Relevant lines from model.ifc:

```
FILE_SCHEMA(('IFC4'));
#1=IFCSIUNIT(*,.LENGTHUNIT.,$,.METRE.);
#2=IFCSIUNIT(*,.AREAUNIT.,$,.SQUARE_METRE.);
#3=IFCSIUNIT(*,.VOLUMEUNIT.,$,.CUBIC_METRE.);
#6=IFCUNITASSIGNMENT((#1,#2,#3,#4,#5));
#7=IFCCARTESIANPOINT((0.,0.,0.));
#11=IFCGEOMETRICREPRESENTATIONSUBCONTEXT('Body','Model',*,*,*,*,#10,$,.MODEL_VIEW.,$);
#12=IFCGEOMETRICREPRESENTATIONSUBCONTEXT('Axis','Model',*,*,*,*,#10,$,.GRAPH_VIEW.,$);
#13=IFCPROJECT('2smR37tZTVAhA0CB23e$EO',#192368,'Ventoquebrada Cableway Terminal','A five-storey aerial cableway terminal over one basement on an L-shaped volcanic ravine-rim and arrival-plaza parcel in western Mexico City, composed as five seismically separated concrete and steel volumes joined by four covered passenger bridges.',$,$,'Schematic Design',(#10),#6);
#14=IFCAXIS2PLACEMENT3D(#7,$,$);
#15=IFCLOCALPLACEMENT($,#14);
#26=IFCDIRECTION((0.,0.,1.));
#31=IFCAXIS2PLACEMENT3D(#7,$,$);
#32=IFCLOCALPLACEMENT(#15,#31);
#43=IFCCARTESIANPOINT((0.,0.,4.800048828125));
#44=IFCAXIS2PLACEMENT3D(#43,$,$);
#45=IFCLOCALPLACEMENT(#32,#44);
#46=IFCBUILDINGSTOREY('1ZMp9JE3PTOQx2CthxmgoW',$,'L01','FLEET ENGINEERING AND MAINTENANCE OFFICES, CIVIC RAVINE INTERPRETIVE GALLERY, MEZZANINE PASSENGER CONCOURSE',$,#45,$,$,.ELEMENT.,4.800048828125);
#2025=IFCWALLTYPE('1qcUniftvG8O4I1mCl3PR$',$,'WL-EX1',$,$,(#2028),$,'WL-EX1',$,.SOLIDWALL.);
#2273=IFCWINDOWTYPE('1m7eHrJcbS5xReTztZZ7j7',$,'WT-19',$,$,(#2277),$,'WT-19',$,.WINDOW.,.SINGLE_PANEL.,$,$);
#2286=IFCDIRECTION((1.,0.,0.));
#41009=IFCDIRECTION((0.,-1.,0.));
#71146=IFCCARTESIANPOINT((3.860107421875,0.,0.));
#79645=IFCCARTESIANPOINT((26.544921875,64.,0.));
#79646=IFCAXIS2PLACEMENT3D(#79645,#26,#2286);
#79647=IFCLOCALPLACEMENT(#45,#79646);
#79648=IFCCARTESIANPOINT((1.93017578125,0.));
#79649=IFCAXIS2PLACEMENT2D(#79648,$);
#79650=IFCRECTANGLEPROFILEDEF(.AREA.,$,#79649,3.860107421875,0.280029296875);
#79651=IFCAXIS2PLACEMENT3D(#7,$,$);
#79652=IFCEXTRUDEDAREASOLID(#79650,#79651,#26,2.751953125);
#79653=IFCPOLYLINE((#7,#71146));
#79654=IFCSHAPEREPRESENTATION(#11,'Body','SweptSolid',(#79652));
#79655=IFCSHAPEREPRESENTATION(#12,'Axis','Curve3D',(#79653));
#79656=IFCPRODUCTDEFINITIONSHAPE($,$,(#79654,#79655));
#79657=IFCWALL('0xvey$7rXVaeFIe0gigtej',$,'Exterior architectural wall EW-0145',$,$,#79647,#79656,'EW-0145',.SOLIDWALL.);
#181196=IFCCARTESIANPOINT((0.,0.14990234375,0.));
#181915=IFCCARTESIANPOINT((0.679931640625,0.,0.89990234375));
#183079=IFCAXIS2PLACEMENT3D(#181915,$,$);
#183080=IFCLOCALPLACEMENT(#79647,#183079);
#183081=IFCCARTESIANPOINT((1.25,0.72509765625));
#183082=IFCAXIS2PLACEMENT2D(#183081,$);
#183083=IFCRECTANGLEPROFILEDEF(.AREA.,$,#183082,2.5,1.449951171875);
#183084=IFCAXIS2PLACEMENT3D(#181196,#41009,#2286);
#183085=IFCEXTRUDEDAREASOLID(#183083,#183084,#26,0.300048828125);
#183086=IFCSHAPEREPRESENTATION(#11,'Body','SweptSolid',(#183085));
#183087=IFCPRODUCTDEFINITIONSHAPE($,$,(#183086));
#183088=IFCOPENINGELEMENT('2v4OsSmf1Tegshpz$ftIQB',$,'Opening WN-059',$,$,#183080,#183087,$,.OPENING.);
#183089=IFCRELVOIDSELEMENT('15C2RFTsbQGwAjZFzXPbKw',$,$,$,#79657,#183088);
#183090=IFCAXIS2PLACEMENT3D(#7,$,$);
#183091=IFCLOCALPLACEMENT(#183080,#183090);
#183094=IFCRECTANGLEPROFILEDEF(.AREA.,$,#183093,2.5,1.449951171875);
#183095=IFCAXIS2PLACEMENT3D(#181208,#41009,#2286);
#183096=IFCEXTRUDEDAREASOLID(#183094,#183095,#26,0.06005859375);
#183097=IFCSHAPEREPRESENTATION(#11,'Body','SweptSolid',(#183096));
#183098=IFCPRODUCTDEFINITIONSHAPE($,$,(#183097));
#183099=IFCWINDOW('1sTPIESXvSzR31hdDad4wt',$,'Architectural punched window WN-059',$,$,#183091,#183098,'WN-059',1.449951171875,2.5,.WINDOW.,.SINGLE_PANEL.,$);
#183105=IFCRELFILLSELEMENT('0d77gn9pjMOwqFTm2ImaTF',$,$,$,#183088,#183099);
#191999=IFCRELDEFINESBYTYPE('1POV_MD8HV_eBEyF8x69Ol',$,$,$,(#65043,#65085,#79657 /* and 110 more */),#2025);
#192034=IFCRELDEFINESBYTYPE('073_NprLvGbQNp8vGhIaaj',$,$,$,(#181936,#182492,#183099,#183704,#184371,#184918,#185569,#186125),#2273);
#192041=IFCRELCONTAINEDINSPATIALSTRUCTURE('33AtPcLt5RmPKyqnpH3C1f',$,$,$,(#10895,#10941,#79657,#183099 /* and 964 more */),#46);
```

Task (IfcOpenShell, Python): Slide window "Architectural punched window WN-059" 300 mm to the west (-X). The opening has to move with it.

```python
import ifcopenshell
import ifcopenshell.api.geometry
import ifcopenshell.util.placement
import ifcopenshell.util.unit

model = ifcopenshell.open("model.ifc")
unit_scale = ifcopenshell.util.unit.calculate_unit_scale(model)

window = model.by_id(183099)
opening = window.FillsVoids[0].RelatingOpeningElement
wall = opening.VoidsElements[0].RelatingBuildingElement

wall_matrix = ifcopenshell.util.placement.get_local_placement(wall.ObjectPlacement)
shift = wall_matrix[:3, 0] * -0.3 / unit_scale
before = ifcopenshell.util.placement.get_local_placement(window.ObjectPlacement)[:3, 3].copy()

# The window is placed relative to its opening, so it follows when the opening moves.
matrix = ifcopenshell.util.placement.get_local_placement(opening.ObjectPlacement)
matrix[:3, 3] += shift
ifcopenshell.api.geometry.edit_object_placement(
    model, product=opening, matrix=matrix, is_si=False, should_transform_children=True
)

after = ifcopenshell.util.placement.get_local_placement(window.ObjectPlacement)[:3, 3]
print("window moved by", (after - before).round(3) + 0.0)

model.write("model_v2.ifc")
```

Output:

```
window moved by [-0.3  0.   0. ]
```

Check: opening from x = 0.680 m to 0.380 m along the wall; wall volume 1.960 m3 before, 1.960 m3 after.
